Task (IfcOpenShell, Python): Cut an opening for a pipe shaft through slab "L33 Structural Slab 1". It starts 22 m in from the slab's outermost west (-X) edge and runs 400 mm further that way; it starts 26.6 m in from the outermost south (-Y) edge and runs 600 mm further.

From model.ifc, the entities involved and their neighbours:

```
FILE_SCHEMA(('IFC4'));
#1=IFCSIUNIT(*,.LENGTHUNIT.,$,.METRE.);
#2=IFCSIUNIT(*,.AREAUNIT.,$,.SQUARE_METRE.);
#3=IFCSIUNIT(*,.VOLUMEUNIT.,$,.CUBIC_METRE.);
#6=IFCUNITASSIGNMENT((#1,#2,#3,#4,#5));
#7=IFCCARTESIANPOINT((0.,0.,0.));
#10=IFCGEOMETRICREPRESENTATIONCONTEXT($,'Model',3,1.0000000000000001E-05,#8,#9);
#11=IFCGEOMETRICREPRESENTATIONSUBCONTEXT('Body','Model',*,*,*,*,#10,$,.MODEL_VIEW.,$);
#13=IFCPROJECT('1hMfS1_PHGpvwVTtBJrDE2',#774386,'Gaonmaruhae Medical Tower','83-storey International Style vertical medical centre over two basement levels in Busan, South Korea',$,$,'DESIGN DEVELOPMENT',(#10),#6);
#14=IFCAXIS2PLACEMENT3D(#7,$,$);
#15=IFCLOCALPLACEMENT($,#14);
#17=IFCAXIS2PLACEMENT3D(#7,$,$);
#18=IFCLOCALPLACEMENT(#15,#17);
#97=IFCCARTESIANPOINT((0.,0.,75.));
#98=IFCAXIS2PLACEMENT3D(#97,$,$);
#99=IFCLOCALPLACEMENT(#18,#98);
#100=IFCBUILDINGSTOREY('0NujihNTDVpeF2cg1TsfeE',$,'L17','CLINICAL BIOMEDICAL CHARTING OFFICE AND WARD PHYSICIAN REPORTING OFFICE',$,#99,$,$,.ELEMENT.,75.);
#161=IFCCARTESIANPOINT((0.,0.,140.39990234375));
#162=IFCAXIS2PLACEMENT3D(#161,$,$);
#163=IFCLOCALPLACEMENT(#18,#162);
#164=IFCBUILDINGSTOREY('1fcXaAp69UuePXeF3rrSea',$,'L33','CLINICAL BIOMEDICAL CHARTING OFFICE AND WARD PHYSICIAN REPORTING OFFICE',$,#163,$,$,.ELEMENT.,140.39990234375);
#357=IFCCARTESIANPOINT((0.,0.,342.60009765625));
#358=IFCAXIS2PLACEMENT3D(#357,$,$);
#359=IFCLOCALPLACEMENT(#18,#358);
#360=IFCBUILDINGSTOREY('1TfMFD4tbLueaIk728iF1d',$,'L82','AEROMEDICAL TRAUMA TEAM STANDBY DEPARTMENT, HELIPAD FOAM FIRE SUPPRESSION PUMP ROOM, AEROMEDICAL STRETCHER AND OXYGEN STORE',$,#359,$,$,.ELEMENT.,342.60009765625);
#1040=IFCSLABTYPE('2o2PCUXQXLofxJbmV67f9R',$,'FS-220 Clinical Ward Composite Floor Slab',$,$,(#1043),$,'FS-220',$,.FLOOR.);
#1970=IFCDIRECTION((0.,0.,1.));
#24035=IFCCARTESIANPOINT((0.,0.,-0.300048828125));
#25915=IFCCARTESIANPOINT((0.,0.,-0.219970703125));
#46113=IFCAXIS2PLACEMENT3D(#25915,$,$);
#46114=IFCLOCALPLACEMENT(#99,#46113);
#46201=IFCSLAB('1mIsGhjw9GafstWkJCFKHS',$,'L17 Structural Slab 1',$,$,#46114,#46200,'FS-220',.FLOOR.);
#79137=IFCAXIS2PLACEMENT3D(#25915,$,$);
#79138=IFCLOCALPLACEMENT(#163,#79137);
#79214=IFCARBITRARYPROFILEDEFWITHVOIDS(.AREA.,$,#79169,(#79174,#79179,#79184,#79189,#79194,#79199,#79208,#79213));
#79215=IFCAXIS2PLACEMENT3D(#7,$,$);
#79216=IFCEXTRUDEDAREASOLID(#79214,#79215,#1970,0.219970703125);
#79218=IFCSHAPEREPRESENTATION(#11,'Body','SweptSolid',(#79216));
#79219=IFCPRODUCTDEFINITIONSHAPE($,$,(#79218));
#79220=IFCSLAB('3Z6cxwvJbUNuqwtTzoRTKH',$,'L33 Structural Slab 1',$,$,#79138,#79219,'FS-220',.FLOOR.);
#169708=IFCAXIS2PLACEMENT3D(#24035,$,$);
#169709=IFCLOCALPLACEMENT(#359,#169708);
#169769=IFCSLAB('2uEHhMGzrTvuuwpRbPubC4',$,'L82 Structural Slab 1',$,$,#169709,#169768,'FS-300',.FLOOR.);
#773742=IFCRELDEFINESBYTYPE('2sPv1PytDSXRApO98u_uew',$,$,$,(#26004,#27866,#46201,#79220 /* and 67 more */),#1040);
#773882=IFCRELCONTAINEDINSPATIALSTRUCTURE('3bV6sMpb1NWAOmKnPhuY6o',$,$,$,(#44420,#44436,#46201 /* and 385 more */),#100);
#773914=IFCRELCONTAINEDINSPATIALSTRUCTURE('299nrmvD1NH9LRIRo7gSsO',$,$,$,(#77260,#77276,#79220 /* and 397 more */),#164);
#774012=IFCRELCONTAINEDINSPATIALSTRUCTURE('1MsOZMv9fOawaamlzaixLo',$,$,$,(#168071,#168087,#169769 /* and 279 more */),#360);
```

```python
import numpy as np
import ifcopenshell
import ifcopenshell.api.feature
import ifcopenshell.api.geometry
import ifcopenshell.api.root
import ifcopenshell.geom
import ifcopenshell.util.placement
import ifcopenshell.util.representation
import ifcopenshell.util.shape
import ifcopenshell.util.unit

model = ifcopenshell.open("model.ifc")
unit_scale = ifcopenshell.util.unit.calculate_unit_scale(model)
settings = ifcopenshell.geom.settings()


def volume(element):
    """Net volume in cubic metres, openings subtracted."""
    shape = ifcopenshell.geom.create_shape(settings, element)
    return ifcopenshell.util.shape.get_volume(shape.geometry)


slab = model.by_guid("3Z6cxwvJbUNuqwtTzoRTKH")
before = volume(slab)

# Extent in the slab's own axes, in metres. The edges named are its -X and -Y sides.
slab_shape = ifcopenshell.geom.create_shape(settings, slab)
vertices = ifcopenshell.util.shape.get_vertices(slab_shape.geometry)
x_min, y_min, bottom = vertices.min(axis=0)
top = vertices[:, 2].max()

opening = ifcopenshell.api.root.create_entity(model, ifc_class="IfcOpeningElement", name="Pipe shaft opening", predefined_type="OPENING")
context = ifcopenshell.util.representation.get_context(model, "Model", "Body", "MODEL_VIEW")
width, depth = 0.4, 0.6
outline = [(0.0, 0.0), (width, 0.0), (width, depth), (0.0, depth), (0.0, 0.0)]
# Overshoot both faces by 50 mm so the cut is clean.
shape = ifcopenshell.api.geometry.add_slab_representation(
    model, context=context, depth=top - bottom + 0.1, polyline=outline
)
ifcopenshell.api.geometry.assign_representation(model, product=opening, representation=shape)

matrix = ifcopenshell.util.placement.get_local_placement(slab.ObjectPlacement)
matrix[:, 3] = matrix @ np.append(np.array([x_min + 22, y_min + 26.6, bottom - 0.05]) / unit_scale, 1.0)
ifcopenshell.api.geometry.edit_object_placement(model, product=opening, matrix=matrix, is_si=False)
ifcopenshell.api.feature.add_feature(model, feature=opening, element=slab)

after = volume(slab)

print(f"slab volume {before:.3f} -> {after:.3f} m3")

model.write("model-out.ifc")
```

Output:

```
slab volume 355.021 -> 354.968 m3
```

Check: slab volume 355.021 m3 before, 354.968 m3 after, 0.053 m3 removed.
